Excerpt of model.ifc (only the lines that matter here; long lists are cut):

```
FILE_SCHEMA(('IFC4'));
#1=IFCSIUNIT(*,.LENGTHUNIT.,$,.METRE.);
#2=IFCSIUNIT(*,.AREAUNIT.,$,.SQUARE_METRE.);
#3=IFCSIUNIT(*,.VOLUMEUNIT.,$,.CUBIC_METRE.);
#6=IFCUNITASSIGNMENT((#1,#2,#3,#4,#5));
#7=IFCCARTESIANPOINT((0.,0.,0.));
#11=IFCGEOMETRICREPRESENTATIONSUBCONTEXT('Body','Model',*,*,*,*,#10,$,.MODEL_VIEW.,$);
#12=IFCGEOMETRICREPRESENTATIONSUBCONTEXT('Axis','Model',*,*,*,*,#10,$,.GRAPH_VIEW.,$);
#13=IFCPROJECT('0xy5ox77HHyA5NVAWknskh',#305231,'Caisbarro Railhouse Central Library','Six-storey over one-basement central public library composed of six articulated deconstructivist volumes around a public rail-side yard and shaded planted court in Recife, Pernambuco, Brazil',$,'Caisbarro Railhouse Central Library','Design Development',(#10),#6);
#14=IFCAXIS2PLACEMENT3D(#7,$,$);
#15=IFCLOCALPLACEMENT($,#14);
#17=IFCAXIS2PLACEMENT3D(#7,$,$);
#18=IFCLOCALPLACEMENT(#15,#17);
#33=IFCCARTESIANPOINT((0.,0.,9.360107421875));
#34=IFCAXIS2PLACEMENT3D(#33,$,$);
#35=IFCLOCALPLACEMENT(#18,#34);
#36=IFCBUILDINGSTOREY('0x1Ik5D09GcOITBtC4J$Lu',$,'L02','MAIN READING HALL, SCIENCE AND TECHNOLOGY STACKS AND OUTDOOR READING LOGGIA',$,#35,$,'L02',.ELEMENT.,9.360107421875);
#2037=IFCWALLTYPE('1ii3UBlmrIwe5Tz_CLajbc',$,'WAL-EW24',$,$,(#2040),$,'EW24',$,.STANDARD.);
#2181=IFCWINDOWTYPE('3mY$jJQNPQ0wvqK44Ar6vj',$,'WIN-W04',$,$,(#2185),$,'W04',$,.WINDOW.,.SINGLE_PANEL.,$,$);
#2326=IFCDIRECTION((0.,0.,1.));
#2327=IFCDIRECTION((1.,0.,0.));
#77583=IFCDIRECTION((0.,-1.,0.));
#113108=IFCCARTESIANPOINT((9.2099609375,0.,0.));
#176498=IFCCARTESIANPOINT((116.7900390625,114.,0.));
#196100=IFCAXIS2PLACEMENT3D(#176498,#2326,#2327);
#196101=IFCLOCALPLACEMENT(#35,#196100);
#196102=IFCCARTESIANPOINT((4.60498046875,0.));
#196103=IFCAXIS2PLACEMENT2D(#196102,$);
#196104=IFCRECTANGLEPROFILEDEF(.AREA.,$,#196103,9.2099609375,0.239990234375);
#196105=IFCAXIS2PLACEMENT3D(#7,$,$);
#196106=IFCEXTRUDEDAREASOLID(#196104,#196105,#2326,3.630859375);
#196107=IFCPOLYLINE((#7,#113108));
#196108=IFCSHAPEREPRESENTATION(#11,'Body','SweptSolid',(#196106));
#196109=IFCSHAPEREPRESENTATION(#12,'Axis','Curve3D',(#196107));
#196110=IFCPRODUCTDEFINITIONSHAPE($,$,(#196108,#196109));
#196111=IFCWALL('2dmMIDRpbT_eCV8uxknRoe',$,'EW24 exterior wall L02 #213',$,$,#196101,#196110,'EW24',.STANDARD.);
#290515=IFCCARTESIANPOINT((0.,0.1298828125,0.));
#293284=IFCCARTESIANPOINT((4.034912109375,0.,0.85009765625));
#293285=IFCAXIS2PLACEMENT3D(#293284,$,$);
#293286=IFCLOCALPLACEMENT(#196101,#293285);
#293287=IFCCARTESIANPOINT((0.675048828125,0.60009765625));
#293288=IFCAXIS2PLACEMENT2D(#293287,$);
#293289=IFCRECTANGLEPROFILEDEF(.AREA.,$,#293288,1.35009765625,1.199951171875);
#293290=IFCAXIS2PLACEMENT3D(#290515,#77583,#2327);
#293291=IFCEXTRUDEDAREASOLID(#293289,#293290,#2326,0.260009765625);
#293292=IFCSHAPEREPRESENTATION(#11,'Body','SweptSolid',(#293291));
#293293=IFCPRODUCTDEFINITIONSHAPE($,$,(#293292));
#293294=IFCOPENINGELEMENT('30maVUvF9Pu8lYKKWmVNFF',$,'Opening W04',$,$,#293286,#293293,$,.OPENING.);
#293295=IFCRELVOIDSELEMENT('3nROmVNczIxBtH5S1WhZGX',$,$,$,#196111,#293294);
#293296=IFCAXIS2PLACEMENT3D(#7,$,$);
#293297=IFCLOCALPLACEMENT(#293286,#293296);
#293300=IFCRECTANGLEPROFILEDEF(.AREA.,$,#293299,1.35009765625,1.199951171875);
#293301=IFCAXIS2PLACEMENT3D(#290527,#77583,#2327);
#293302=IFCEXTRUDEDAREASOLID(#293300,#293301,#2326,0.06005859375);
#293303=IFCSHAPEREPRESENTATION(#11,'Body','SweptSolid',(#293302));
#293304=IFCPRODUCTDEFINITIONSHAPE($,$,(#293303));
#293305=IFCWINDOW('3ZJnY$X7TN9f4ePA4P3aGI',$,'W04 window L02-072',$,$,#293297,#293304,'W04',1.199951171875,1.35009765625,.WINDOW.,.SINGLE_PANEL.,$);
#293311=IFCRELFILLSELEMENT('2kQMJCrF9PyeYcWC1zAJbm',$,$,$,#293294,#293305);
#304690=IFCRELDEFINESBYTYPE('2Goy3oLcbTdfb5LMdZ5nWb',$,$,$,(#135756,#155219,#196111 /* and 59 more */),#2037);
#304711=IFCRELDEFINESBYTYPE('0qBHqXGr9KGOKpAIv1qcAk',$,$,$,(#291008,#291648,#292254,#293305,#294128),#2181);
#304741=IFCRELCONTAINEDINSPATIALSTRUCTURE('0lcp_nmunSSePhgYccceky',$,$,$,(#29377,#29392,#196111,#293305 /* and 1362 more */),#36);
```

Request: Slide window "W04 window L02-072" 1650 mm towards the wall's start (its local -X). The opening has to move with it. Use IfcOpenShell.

```python
import ifcopenshell
import ifcopenshell.api.geometry
import ifcopenshell.util.placement
import ifcopenshell.util.unit

model = ifcopenshell.open("model.ifc")
unit_scale = ifcopenshell.util.unit.calculate_unit_scale(model)

window = model.by_id(293305)
opening = window.FillsVoids[0].RelatingOpeningElement
wall = opening.VoidsElements[0].RelatingBuildingElement

wall_matrix = ifcopenshell.util.placement.get_local_placement(wall.ObjectPlacement)
shift = wall_matrix[:3, 0] * -1.65 / unit_scale
before = ifcopenshell.util.placement.get_local_placement(window.ObjectPlacement)[:3, 3].copy()

# The window is placed relative to its opening, so it follows when the opening moves.
matrix = ifcopenshell.util.placement.get_local_placement(opening.ObjectPlacement)
matrix[:3, 3] += shift
ifcopenshell.api.geometry.edit_object_placement(
    model, product=opening, matrix=matrix, is_si=False, should_transform_children=True
)

after = ifcopenshell.util.placement.get_local_placement(window.ObjectPlacement)[:3, 3]
print("window moved by", (after - before).round(3) + 0.0)

model.write("model-out.ifc")
```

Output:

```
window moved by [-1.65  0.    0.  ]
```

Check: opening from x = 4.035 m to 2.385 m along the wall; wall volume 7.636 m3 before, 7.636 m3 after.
